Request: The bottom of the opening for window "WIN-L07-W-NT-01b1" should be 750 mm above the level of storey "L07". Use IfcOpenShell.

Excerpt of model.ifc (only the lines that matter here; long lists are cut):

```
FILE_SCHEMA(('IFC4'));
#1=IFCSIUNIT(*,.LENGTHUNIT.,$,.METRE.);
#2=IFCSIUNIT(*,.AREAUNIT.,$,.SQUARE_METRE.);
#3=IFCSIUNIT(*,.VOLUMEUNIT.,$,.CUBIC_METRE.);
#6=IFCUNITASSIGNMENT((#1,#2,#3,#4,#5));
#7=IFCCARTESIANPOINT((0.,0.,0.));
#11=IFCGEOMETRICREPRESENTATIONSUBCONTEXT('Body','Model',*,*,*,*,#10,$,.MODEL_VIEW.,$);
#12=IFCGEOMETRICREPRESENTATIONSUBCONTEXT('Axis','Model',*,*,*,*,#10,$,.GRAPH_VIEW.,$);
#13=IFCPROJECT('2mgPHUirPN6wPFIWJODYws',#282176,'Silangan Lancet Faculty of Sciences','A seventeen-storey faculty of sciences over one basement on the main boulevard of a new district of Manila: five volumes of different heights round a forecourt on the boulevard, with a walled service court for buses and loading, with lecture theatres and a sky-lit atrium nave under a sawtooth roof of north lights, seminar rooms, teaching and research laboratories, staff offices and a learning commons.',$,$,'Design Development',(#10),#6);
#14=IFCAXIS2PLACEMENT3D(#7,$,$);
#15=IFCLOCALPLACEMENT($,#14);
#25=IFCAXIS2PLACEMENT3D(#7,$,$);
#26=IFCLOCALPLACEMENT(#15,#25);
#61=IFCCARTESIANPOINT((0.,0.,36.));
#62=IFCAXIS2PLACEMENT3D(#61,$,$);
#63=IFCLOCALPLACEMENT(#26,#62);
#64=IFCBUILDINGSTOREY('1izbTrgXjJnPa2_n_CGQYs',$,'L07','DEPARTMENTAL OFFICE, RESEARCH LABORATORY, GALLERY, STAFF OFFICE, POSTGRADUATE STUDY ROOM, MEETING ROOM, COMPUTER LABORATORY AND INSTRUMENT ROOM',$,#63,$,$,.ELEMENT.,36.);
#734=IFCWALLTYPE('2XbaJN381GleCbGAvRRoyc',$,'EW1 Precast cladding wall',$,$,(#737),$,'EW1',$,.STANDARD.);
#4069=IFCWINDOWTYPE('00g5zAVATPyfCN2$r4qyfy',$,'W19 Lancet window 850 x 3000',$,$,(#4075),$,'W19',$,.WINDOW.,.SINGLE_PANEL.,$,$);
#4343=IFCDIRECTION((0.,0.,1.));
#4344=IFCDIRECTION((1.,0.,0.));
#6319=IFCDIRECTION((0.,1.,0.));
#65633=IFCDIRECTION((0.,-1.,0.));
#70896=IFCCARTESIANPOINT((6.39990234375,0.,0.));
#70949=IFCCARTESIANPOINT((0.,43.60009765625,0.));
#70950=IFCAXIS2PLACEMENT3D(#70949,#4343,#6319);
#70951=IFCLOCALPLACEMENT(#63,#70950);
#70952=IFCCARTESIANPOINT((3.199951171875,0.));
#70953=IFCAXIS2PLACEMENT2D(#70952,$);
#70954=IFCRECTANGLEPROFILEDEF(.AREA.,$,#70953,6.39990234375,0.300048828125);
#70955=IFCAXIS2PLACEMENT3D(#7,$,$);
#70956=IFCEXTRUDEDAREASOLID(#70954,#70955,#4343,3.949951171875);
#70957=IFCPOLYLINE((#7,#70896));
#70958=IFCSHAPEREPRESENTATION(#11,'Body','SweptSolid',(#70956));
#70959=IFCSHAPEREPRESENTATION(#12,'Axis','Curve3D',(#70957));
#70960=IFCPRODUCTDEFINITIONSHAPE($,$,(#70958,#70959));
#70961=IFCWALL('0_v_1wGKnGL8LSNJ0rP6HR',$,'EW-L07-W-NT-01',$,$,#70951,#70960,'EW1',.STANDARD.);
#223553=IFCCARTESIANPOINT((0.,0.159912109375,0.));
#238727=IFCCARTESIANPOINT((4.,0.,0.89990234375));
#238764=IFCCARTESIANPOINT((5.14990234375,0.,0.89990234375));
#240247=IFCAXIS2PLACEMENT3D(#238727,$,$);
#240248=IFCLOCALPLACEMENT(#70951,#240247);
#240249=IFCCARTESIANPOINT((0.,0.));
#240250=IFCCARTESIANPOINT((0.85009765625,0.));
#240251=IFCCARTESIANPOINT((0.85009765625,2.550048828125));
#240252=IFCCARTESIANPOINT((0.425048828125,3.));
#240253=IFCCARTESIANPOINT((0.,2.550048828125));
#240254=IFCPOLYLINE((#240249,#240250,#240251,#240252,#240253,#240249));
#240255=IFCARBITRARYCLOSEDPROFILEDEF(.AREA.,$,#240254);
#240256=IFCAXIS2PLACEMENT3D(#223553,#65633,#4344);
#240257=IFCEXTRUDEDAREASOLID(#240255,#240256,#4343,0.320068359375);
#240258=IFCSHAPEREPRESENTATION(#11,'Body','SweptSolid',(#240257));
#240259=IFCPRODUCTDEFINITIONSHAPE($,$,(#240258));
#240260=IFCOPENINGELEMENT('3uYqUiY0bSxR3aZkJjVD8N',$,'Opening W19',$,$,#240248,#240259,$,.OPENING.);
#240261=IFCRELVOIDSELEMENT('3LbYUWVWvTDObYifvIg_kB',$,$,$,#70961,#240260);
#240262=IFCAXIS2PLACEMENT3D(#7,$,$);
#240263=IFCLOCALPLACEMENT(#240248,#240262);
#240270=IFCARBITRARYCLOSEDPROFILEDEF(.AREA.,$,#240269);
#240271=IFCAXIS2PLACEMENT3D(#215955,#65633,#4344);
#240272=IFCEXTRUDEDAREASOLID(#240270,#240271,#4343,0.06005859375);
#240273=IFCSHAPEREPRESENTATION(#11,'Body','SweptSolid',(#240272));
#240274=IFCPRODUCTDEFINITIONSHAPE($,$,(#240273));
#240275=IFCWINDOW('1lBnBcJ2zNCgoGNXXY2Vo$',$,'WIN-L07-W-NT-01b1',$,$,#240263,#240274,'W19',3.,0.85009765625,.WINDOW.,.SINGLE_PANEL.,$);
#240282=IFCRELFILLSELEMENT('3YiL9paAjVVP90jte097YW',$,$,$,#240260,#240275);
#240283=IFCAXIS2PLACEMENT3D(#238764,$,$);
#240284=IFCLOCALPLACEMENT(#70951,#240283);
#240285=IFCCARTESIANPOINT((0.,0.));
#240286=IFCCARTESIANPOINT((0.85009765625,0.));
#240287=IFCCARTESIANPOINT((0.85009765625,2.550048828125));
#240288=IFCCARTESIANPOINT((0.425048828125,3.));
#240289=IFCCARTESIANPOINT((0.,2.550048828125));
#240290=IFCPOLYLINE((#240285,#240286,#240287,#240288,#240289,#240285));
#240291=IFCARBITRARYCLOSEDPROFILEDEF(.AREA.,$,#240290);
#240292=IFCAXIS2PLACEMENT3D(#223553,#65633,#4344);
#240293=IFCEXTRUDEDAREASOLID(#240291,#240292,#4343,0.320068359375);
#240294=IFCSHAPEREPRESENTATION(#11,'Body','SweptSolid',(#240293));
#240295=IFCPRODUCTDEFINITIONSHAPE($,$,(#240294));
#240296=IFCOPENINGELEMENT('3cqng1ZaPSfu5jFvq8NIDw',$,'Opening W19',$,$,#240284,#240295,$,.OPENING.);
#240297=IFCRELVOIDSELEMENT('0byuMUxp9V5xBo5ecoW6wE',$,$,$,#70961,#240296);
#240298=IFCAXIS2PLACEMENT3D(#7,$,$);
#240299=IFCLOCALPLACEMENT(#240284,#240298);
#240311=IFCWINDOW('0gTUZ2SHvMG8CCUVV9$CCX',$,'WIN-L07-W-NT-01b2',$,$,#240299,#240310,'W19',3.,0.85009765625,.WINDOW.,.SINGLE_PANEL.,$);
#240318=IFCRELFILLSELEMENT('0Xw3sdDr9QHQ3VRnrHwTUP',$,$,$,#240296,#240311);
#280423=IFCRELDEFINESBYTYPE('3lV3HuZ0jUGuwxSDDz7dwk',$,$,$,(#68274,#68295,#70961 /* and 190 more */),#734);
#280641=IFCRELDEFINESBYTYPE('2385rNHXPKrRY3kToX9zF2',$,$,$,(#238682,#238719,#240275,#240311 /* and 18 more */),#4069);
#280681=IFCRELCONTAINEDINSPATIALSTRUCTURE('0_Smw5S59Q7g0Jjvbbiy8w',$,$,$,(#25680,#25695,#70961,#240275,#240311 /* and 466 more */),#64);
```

```python
import numpy as np
import ifcopenshell
import ifcopenshell.api.geometry
import ifcopenshell.geom
import ifcopenshell.util.element
import ifcopenshell.util.placement
import ifcopenshell.util.shape
import ifcopenshell.util.unit

model = ifcopenshell.open("model.ifc")
unit_scale = ifcopenshell.util.unit.calculate_unit_scale(model)

window = model.by_id(240275)
opening = window.FillsVoids[0].RelatingOpeningElement
storey = ifcopenshell.util.element.get_container(window, ifc_class="IfcBuildingStorey")
level = ifcopenshell.util.placement.get_local_placement(storey.ObjectPlacement)[2, 3]

# The opening's origin need not be at the sill, so measure its lowest point.
shape = ifcopenshell.geom.create_shape(ifcopenshell.geom.settings(), opening)
bottom = ifcopenshell.util.shape.get_shape_bottom_elevation(shape, shape.geometry) / unit_scale
dz = level + 0.75 - bottom

shift = np.array([0.0, 0.0, dz])
# The window is placed relative to its opening, so it follows when the opening moves.
matrix = ifcopenshell.util.placement.get_local_placement(opening.ObjectPlacement)
matrix[:3, 3] += shift
ifcopenshell.api.geometry.edit_object_placement(
    model, product=opening, matrix=matrix, is_si=False, should_transform_children=True
)

print(f"moved by {dz * unit_scale:+.3f} m")

model.write("model-out.ifc")
```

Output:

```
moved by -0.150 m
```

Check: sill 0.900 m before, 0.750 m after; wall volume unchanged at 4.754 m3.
